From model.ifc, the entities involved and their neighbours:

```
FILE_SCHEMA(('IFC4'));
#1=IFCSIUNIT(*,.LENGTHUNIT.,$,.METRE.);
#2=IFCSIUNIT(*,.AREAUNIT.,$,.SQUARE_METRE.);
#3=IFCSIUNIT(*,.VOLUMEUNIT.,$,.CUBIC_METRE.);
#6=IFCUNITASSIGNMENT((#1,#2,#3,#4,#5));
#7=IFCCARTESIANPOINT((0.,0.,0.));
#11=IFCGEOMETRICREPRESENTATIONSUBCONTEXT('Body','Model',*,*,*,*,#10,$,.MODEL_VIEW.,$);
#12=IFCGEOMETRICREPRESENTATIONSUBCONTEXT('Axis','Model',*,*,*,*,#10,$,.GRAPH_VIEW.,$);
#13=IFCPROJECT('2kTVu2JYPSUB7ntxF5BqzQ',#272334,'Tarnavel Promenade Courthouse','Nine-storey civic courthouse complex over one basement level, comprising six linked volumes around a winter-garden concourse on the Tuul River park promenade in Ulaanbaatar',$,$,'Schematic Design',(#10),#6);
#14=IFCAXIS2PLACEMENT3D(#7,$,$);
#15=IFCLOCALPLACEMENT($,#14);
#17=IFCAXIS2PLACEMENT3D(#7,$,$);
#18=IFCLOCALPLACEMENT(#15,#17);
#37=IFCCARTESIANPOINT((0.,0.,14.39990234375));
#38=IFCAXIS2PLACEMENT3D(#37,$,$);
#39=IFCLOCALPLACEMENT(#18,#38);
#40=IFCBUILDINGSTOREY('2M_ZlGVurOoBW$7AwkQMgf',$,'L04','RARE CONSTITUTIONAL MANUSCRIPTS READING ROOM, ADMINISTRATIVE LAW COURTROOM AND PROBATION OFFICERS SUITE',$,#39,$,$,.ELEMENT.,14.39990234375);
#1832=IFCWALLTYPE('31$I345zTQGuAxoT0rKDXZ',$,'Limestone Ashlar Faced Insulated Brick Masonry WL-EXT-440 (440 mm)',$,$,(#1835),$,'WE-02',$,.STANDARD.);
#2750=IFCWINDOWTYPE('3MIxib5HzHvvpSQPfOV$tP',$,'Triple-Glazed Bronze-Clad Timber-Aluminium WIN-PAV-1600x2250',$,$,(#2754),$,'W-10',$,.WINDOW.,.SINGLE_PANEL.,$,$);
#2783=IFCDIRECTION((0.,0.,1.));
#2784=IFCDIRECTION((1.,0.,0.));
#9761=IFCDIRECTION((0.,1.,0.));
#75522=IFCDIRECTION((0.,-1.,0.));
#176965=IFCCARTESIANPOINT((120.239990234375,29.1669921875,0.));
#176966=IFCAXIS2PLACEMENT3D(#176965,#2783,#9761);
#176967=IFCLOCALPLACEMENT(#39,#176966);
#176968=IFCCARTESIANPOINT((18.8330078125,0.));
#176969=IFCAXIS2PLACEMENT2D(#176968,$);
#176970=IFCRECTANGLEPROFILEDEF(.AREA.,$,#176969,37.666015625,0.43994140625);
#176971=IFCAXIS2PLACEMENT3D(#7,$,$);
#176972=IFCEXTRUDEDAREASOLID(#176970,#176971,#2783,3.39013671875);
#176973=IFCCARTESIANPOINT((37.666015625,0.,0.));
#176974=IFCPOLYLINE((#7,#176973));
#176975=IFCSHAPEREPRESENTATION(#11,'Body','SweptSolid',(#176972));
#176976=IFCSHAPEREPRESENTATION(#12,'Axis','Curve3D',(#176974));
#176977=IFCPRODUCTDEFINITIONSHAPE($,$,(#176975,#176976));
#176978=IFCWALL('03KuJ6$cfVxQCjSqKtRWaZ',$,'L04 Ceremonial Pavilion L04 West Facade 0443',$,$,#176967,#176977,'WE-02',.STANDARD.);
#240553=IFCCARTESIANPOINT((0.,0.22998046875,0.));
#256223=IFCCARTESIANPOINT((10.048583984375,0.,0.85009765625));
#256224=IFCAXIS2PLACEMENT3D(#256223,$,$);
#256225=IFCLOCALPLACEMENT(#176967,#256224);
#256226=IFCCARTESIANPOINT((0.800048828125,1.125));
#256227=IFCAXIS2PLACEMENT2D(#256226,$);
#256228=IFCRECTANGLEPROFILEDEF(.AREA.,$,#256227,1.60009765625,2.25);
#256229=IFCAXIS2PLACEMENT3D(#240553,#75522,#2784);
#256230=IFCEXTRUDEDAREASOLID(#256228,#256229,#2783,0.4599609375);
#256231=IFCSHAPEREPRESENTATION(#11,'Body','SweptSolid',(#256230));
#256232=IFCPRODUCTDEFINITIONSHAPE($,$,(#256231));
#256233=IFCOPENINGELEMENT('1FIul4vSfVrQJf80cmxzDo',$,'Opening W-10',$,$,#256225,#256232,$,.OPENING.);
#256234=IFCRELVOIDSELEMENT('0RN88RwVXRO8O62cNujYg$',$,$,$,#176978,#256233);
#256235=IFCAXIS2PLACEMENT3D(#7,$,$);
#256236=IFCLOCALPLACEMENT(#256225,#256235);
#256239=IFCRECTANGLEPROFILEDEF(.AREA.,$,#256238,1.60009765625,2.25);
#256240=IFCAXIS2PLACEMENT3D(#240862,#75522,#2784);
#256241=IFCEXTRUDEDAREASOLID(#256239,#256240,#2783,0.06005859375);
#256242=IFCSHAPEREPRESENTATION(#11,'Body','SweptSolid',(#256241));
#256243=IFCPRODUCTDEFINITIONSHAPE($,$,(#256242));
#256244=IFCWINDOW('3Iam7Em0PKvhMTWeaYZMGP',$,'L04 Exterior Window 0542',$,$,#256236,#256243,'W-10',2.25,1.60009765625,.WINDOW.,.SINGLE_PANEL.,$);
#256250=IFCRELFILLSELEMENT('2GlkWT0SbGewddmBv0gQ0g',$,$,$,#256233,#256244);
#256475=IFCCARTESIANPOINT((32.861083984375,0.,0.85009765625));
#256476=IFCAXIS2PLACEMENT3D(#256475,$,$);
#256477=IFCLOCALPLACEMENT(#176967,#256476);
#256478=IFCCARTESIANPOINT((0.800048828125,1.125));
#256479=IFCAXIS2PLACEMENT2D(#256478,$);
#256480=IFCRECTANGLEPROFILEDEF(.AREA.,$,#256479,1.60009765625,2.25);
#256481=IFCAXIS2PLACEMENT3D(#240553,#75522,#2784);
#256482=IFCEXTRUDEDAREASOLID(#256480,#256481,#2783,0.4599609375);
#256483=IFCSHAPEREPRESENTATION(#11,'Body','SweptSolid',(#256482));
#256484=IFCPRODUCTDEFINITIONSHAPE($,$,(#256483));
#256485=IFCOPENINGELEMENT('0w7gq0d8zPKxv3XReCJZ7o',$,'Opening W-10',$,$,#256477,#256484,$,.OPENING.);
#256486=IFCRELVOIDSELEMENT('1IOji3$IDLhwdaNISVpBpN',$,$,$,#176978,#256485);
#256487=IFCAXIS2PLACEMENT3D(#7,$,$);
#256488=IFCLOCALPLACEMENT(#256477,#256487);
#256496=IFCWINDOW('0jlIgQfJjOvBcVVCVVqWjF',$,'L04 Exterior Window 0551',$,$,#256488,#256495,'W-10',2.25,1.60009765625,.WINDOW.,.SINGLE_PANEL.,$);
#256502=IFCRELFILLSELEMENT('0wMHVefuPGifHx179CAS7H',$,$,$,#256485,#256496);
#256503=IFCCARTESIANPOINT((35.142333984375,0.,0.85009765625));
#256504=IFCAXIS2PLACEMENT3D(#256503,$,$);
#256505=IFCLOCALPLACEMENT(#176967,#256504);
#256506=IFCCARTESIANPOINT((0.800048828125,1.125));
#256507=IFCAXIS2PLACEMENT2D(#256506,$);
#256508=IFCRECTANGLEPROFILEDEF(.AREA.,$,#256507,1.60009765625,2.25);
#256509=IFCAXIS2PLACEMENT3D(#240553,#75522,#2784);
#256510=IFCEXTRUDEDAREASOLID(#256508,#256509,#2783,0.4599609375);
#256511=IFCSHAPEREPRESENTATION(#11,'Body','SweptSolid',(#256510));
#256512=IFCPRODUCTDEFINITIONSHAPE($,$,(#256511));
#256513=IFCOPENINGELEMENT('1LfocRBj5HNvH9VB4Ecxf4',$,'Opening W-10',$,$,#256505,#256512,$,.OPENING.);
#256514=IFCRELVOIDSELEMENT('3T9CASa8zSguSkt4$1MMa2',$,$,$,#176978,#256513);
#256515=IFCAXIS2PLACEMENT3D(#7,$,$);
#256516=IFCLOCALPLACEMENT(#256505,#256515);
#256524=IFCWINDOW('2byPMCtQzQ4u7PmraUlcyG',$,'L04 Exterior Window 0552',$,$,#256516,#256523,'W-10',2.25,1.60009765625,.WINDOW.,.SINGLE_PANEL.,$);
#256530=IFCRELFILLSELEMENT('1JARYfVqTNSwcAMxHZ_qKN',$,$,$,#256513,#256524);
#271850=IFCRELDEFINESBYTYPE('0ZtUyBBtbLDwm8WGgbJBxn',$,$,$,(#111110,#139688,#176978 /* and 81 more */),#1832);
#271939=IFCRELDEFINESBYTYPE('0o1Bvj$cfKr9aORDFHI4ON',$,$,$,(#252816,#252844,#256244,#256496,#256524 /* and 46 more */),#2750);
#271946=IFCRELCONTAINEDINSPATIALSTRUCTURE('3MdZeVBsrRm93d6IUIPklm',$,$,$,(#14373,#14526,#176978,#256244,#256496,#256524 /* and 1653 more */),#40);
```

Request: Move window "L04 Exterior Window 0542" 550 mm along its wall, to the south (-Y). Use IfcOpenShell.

```python
import ifcopenshell
import ifcopenshell.api.geometry
import ifcopenshell.util.placement
import ifcopenshell.util.unit

model = ifcopenshell.open("model.ifc")
unit_scale = ifcopenshell.util.unit.calculate_unit_scale(model)

window = model.by_id(256244)
opening = window.FillsVoids[0].RelatingOpeningElement
wall = opening.VoidsElements[0].RelatingBuildingElement

wall_matrix = ifcopenshell.util.placement.get_local_placement(wall.ObjectPlacement)
shift = wall_matrix[:3, 0] * -0.55 / unit_scale
before = ifcopenshell.util.placement.get_local_placement(window.ObjectPlacement)[:3, 3].copy()

# The window is placed relative to its opening, so it follows when the opening moves.
matrix = ifcopenshell.util.placement.get_local_placement(opening.ObjectPlacement)
matrix[:3, 3] += shift
ifcopenshell.api.geometry.edit_object_placement(
    model, product=opening, matrix=matrix, is_si=False, should_transform_children=True
)

after = ifcopenshell.util.placement.get_local_placement(window.ObjectPlacement)[:3, 3]
print("window moved by", (after - before).round(3) + 0.0)

model.write("model-out.ifc")
```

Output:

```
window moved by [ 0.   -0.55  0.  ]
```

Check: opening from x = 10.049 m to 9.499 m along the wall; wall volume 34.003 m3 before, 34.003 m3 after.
